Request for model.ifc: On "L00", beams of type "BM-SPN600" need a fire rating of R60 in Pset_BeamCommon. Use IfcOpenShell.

First a look at what the model holds.

```python
import ifcopenshell
import ifcopenshell.util.element

model = ifcopenshell.open("model.ifc")
print(model.schema)
storey = next(s for s in model.by_type("IfcBuildingStorey") if s.Name == "L00")
beams = [e for e in ifcopenshell.util.element.get_decomposition(storey) if e.is_a("IfcBeam")]
seen = {}
for e in beams:
    element_type = ifcopenshell.util.element.get_type(e)
    key = (element_type.Name if element_type != e and element_type else None, ifcopenshell.util.element.get_pset(e, "Pset_BeamCommon", "FireRating"))
    seen[key] = seen.get(key, 0) + 1
for (name, value), count in sorted(seen.items(), key=str):
    print(count, "x", name, "|", value)
```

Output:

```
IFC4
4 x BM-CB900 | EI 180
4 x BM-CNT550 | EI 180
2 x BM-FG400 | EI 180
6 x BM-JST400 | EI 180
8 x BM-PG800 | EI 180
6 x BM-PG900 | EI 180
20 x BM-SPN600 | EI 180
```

```python
import ifcopenshell
import ifcopenshell.api.pset
import ifcopenshell.util.element

model = ifcopenshell.open("model.ifc")

storey = next(s for s in model.by_type("IfcBuildingStorey") if s.Name == "L00")
beams = [e for e in ifcopenshell.util.element.get_decomposition(storey) if e.is_a("IfcBeam")]

count = 0
for e in beams:
    element_type = ifcopenshell.util.element.get_type(e)
    if element_type in (None, e) or element_type.Name != "BM-SPN600":
        continue
    # add_pset returns the element's existing set when there is one.
    pset = ifcopenshell.api.pset.add_pset(model, product=e, name="Pset_BeamCommon")
    ifcopenshell.api.pset.edit_pset(model, pset=pset, properties={"FireRating": "R60"})
    count += 1

print(count, "beams updated")

model.write("model_rev.ifc")
```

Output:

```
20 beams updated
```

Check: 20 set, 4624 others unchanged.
